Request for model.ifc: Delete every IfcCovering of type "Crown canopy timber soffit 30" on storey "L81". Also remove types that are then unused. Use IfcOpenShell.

First a look at what the model holds.

```python
import ifcopenshell
import ifcopenshell.util.element

model = ifcopenshell.open("model.ifc")
print(model.schema)
storey = next(s for s in model.by_type("IfcBuildingStorey") if s.Name == "L81")
coverings = [e for e in ifcopenshell.util.element.get_decomposition(storey) if e.is_a("IfcCovering")]
seen = {}
for e in coverings:
    element_type = ifcopenshell.util.element.get_type(e)
    name = element_type.Name if element_type not in (None, e) else None
    seen[name] = seen.get(name, 0) + 1
for name, count in sorted(seen.items(), key=str):
    print(count, "x", name)
```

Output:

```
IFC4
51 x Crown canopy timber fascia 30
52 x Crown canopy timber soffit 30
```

```python
import ifcopenshell
import ifcopenshell.api.root
import ifcopenshell.util.element

model = ifcopenshell.open("model.ifc")

storey = next(s for s in model.by_type("IfcBuildingStorey") if s.Name == "L81")
coverings = [e for e in ifcopenshell.util.element.get_decomposition(storey) if e.is_a("IfcCovering")]
targets = [e for e in coverings if (t := ifcopenshell.util.element.get_type(e)) not in (None, e) and t.Name == "Crown canopy timber soffit 30"]
types = {ifcopenshell.util.element.get_type(e) for e in targets} - {None, *targets}

for e in targets:
    ifcopenshell.api.root.remove_product(model, product=e)
print(len(targets), "removed")

unused = [t for t in types if not ifcopenshell.util.element.get_types(t)]
for t in unused:
    ifcopenshell.api.root.remove_product(model, product=t)
print(len(unused), "unused types removed")

model.write("model-out.ifc")
```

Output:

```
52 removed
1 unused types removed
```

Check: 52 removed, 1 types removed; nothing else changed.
